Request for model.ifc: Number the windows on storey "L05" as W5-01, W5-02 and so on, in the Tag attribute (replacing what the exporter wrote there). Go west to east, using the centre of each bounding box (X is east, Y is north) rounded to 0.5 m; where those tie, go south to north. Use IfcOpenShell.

First a look at what the model holds.

```python
import ifcopenshell
import ifcopenshell.util.element
import ifcopenshell.util.placement

model = ifcopenshell.open("model.ifc")
print(model.schema)
storey = next(s for s in model.by_type("IfcBuildingStorey") if s.Name == "L05")
windows = [e for e in ifcopenshell.util.element.get_decomposition(storey) if e.is_a("IfcWindow")]
for e in sorted(windows, key=lambda e: e.id()):
    origin = ifcopenshell.util.placement.get_local_placement(e.ObjectPlacement)[:3, 3]
    print(e.id(), e.Tag, e.Name, origin.round(2) + 0.0, sep=" | ")
```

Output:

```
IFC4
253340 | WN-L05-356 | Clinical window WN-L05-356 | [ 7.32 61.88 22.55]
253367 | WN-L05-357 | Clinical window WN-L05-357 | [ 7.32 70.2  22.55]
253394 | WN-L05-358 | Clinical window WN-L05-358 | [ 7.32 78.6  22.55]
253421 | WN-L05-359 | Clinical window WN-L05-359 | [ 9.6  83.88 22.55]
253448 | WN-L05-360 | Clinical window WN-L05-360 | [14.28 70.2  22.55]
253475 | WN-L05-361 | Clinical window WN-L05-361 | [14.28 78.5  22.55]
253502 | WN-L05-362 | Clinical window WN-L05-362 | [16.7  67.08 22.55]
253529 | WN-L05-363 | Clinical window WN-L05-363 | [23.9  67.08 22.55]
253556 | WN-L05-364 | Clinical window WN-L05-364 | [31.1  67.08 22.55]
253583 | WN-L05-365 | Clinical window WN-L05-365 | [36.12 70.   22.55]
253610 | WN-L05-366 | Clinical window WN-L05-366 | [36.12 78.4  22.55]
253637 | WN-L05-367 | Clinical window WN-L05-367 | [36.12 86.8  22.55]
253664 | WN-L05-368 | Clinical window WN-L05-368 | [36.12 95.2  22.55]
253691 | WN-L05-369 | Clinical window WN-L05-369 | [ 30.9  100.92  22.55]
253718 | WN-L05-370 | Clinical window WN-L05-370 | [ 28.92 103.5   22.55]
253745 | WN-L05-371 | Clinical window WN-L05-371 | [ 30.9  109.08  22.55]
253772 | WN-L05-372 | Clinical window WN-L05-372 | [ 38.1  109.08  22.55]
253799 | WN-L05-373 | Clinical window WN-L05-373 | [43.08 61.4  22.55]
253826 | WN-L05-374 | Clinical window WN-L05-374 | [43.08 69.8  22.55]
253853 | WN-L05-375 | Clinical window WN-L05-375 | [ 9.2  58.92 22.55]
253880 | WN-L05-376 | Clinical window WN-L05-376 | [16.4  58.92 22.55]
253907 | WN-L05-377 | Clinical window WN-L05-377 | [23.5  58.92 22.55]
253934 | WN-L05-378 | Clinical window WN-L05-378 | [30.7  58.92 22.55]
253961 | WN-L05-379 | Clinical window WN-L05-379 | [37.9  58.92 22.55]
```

```python
import ifcopenshell
import ifcopenshell.geom
import ifcopenshell.util.element
import ifcopenshell.util.shape

model = ifcopenshell.open("model.ifc")
settings = ifcopenshell.geom.settings()
settings.set("use-world-coords", True)


def centre(element):
    shape = ifcopenshell.geom.create_shape(settings, element)
    return ifcopenshell.util.shape.get_bbox_centroid(shape.geometry)


storey = next(s for s in model.by_type("IfcBuildingStorey") if s.Name == "L05")
windows = [e for e in ifcopenshell.util.element.get_decomposition(storey) if e.is_a("IfcWindow")]

# Insertion points can sit at a corner or the storey origin, so sort by the geometry (in metres).
centres = {e: centre(e) for e in windows}
windows.sort(key=lambda e: (round(centres[e][0] / 0.5), centres[e][1]))

for i, e in enumerate(windows, start=1):
    number = f"W5-{i:02d}"
    e.Tag = number
    print(e.id(), number)

model.write("model_edited.ifc")
```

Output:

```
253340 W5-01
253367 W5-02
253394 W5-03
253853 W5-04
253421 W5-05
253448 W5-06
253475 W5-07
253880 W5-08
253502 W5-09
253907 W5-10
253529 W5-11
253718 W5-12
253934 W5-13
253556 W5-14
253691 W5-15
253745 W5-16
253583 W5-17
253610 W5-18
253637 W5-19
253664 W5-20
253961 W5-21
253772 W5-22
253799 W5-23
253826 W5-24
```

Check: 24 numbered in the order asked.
